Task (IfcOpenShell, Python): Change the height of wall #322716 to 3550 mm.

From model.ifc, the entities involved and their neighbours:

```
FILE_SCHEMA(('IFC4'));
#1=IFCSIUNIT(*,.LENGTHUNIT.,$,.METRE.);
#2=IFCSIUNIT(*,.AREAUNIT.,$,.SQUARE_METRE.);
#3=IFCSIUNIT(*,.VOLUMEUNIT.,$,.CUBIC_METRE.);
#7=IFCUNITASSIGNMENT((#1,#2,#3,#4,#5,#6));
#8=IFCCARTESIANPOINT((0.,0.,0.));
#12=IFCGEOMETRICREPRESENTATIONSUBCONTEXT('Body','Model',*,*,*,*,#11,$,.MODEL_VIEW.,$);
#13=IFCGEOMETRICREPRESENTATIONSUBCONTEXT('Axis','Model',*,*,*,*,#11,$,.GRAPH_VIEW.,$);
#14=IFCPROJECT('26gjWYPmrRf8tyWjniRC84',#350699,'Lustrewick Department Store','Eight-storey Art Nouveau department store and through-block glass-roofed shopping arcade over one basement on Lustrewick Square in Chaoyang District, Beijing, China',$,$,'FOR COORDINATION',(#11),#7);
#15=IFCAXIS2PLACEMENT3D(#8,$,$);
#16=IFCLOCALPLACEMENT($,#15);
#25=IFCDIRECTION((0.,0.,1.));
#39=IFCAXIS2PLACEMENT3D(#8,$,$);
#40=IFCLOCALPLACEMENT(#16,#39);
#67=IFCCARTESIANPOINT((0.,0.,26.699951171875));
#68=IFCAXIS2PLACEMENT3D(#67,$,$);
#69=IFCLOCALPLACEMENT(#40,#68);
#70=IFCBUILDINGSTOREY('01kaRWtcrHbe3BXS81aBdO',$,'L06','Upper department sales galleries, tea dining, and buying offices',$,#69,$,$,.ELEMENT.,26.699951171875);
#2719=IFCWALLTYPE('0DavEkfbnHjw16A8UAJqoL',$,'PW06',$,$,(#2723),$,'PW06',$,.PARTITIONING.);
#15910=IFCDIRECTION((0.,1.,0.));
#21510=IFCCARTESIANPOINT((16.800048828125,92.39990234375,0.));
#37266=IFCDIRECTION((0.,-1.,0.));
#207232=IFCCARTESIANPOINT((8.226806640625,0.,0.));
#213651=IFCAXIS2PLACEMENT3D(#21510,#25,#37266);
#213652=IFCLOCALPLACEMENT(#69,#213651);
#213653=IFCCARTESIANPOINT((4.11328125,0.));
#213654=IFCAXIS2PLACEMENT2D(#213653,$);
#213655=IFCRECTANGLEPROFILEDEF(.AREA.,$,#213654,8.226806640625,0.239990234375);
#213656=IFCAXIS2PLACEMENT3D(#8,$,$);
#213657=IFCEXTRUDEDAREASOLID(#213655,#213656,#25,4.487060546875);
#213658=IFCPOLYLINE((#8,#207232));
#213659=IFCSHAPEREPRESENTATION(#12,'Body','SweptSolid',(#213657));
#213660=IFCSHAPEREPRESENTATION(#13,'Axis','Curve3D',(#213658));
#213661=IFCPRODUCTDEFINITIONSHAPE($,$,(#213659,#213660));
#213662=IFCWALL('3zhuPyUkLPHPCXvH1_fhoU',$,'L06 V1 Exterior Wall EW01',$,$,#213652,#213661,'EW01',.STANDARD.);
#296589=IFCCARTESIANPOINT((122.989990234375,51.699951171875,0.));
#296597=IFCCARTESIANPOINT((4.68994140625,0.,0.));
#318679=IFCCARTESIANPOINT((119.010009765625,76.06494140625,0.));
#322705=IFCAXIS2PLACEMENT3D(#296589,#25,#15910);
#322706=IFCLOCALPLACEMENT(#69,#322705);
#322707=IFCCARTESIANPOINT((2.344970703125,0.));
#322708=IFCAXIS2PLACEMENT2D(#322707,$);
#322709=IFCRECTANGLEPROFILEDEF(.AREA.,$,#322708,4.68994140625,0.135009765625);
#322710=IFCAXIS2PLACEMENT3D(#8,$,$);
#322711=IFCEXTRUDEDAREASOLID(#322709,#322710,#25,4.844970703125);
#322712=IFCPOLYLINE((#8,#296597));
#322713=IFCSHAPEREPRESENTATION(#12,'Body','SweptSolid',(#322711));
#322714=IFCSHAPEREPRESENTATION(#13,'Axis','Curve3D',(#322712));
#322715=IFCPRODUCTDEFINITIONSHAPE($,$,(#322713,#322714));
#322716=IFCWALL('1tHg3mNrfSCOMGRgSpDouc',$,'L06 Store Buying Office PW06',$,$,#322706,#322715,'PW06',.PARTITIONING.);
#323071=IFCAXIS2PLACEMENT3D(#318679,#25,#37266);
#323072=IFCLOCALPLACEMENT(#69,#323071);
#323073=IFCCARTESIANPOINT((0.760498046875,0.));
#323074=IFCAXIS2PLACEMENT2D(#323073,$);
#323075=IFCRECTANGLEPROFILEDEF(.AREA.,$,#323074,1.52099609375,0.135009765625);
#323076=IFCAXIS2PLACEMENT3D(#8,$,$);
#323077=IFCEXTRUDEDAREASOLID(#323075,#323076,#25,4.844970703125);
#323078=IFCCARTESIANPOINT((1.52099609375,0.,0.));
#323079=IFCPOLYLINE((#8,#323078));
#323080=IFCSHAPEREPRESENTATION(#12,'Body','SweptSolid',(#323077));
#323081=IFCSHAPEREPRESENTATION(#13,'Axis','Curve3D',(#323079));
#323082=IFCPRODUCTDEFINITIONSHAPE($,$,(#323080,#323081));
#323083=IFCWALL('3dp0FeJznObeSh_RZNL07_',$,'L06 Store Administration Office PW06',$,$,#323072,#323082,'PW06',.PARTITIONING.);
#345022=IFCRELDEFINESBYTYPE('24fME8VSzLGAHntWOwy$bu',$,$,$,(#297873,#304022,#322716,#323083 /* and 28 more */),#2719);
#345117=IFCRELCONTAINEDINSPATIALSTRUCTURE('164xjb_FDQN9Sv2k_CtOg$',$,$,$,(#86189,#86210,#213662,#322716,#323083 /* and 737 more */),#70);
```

```python
import ifcopenshell
import ifcopenshell.geom
import ifcopenshell.util.representation
import ifcopenshell.util.shape
import ifcopenshell.util.unit

model = ifcopenshell.open("model.ifc")
unit_scale = ifcopenshell.util.unit.calculate_unit_scale(model)
settings = ifcopenshell.geom.settings()


def volume(element):
    """Net volume in cubic metres, openings subtracted."""
    shape = ifcopenshell.geom.create_shape(settings, element)
    return ifcopenshell.util.shape.get_volume(shape.geometry)


wall = model.by_guid("1tHg3mNrfSCOMGRgSpDouc")
before = volume(wall)

body = ifcopenshell.util.representation.get_representation(wall, "Model", "Body")
solid = body.Items[0]
old_height = solid.Depth
solid.Depth = 3.55 / unit_scale
after = volume(wall)

print(f"height {old_height:g} -> {solid.Depth:g}, volume {before:.3f} -> {after:.3f} m3")

model.write("model_updated.ifc")
```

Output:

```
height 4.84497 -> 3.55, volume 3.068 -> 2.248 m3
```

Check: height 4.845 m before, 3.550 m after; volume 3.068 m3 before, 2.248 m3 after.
